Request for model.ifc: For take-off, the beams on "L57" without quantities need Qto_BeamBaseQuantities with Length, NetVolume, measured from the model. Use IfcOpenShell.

First a look at what the model holds.

```python
import ifcopenshell
import ifcopenshell.util.element
import ifcopenshell.util.unit

model = ifcopenshell.open("model.ifc")
print(model.schema)
for unit_type in ("LENGTHUNIT", "AREAUNIT", "VOLUMEUNIT"):
    print(unit_type, ifcopenshell.util.unit.calculate_unit_scale(model, unit_type))
storey = next(s for s in model.by_type("IfcBuildingStorey") if s.Name == "L57")
beams = [e for e in ifcopenshell.util.element.get_decomposition(storey) if e.is_a("IfcBeam")]
for e in sorted(beams, key=lambda e: e.id()):
    print(e.id(), e.is_a(), e.Name, list(ifcopenshell.util.element.get_psets(e, qtos_only=True)), sep=" | ")
```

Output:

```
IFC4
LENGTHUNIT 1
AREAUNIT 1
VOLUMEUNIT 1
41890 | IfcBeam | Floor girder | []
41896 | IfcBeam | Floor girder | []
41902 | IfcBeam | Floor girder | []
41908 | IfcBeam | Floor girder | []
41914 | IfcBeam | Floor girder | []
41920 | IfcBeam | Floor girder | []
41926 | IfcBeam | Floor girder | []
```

```python
import ifcopenshell
import ifcopenshell.api.pset
import ifcopenshell.geom
import ifcopenshell.util.element
import ifcopenshell.util.shape
import ifcopenshell.util.unit

model = ifcopenshell.open("model.ifc")
unit_scale = ifcopenshell.util.unit.calculate_unit_scale(model)
volume_scale = ifcopenshell.util.unit.calculate_unit_scale(model, "VOLUMEUNIT")
settings = ifcopenshell.geom.settings()

storey = next(s for s in model.by_type("IfcBuildingStorey") if s.Name == "L57")
beams = [e for e in ifcopenshell.util.element.get_decomposition(storey) if e.is_a("IfcBeam")]

for e in sorted(beams, key=lambda e: e.id()):
    if ifcopenshell.util.element.get_psets(e, qtos_only=True, should_inherit=False):
        continue
    # Geometry comes back in metres, in the element's own axes.
    shape = ifcopenshell.geom.create_shape(settings, e)
    values = {
        "Length": ifcopenshell.util.shape.get_max_xyz(shape.geometry) / unit_scale,
        "NetVolume": ifcopenshell.util.shape.get_volume(shape.geometry) / volume_scale,
    }
    qto = ifcopenshell.api.pset.add_qto(model, product=e, name="Qto_BeamBaseQuantities")
    ifcopenshell.api.pset.edit_qto(model, qto=qto, properties=values)
    print(e.id(), {k: round(v, 3) for k, v in values.items()})

model.write("model_v2.ifc")
```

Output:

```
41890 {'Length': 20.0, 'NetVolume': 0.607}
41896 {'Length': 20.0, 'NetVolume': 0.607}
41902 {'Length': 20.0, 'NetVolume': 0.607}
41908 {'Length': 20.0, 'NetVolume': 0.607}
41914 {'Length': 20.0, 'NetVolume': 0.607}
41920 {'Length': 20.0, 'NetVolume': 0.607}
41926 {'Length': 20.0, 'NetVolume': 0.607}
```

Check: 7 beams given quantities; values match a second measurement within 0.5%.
